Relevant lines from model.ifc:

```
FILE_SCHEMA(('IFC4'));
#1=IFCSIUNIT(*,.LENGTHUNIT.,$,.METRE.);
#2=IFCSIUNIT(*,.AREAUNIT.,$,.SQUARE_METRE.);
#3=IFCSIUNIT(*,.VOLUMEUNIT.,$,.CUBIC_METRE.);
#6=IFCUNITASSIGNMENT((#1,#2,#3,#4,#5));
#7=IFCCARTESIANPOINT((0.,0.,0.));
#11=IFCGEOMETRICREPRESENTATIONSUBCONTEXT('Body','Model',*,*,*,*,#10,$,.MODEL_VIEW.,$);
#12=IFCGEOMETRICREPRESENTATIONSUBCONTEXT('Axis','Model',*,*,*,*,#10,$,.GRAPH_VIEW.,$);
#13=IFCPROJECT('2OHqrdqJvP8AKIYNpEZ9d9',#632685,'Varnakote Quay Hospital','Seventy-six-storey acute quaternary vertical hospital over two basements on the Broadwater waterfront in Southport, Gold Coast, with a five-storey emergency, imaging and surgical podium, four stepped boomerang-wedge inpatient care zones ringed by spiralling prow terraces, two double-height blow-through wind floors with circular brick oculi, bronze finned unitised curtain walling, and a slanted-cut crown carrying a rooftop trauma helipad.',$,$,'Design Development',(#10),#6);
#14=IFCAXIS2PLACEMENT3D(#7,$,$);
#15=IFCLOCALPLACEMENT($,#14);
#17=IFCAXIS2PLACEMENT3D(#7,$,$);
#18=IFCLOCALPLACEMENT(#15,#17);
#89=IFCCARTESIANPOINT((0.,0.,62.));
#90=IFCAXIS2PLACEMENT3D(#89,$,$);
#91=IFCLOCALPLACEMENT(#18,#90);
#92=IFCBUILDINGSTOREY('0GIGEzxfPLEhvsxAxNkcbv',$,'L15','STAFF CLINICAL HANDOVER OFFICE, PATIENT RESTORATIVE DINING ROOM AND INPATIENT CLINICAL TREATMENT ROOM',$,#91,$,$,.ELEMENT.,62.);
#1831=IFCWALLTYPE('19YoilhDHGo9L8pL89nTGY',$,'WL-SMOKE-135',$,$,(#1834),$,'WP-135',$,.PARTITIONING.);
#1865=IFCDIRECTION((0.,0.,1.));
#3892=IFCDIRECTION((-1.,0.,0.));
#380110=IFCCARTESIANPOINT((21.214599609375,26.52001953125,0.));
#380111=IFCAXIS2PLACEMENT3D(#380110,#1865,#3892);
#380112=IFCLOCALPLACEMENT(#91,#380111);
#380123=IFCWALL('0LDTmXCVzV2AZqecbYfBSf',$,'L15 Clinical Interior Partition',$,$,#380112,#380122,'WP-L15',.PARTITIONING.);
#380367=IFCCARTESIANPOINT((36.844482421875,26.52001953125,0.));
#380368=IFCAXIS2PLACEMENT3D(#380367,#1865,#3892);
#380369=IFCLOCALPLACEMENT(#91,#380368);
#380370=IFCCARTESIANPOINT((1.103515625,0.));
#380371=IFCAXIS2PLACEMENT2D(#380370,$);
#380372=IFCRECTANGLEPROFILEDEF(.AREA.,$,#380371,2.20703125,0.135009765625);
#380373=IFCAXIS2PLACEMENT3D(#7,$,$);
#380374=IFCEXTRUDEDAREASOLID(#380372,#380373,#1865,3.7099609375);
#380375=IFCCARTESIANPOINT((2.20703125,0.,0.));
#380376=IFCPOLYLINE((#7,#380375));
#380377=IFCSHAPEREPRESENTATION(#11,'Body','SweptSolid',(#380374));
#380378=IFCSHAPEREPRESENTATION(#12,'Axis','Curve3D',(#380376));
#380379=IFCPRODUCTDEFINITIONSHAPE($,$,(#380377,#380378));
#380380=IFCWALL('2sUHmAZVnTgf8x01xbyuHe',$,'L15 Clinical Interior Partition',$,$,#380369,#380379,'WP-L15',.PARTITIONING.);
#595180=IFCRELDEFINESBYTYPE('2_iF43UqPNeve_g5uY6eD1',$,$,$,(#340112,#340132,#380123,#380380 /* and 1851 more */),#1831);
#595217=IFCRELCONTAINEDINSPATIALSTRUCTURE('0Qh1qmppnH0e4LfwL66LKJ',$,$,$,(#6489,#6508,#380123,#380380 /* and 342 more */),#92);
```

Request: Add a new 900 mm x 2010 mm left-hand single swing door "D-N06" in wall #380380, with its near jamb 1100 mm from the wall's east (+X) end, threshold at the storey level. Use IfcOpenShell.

```python
import numpy as np
import ifcopenshell
import ifcopenshell.api.feature
import ifcopenshell.api.geometry
import ifcopenshell.api.root
import ifcopenshell.api.spatial
import ifcopenshell.geom
import ifcopenshell.util.element
import ifcopenshell.util.placement
import ifcopenshell.util.representation
import ifcopenshell.util.shape
import ifcopenshell.util.unit

model = ifcopenshell.open("model.ifc")
unit_scale = ifcopenshell.util.unit.calculate_unit_scale(model)
settings = ifcopenshell.geom.settings()


def volume(element):
    """Net volume in cubic metres, openings subtracted."""
    shape = ifcopenshell.geom.create_shape(settings, element)
    return ifcopenshell.util.shape.get_volume(shape.geometry)


wall = model.by_id(380380)
storey = ifcopenshell.util.element.get_container(wall, ifc_class="IfcBuildingStorey")
context = ifcopenshell.util.representation.get_context(model, "Model", "Body", "MODEL_VIEW")
before = volume(wall)

width, height, from_end, sill = 0.9, 2.01, 1.1, 0.0  # metres

# The wall runs along its own X axis, and the end named is its -X end.
wall_shape = ifcopenshell.geom.create_shape(settings, wall)
x, y, z = ifcopenshell.util.shape.get_vertices(wall_shape.geometry).T
start = x.min() + from_end
face, thickness = float(y.min()), float(y.max() - y.min())
wall_matrix = ifcopenshell.util.placement.get_local_placement(wall.ObjectPlacement)
level = ifcopenshell.util.placement.get_local_placement(storey.ObjectPlacement)[2, 3]


def in_wall(x, y):
    """Placement at x, y metres in the wall's axes, at sill height."""
    matrix = wall_matrix.copy()
    matrix[:, 3] = wall_matrix @ np.array([x / unit_scale, y / unit_scale, 0.0, 1.0])
    matrix[2, 3] = level + sill / unit_scale
    return matrix


# Opening: a box that overshoots both wall faces by 50 mm.
opening = ifcopenshell.api.root.create_entity(model, ifc_class="IfcOpeningElement", predefined_type="OPENING")
box = ifcopenshell.api.geometry.add_wall_representation(
    model, context=context, length=width, height=height, thickness=thickness + 0.1
)
ifcopenshell.api.geometry.assign_representation(model, product=opening, representation=box)
ifcopenshell.api.geometry.edit_object_placement(model, product=opening, matrix=in_wall(start, face - 0.05), is_si=False)
ifcopenshell.api.feature.add_feature(model, feature=opening, element=wall)

door = ifcopenshell.api.root.create_entity(model, ifc_class="IfcDoor", name="D-N06", predefined_type="DOOR")
door.OverallWidth, door.OverallHeight = width / unit_scale, height / unit_scale
door.OperationType = "SINGLE_SWING_LEFT"
body = ifcopenshell.api.geometry.add_door_representation(
    model,
    context=context,
    overall_width=door.OverallWidth,
    overall_height=door.OverallHeight,
    operation_type="SINGLE_SWING_LEFT",
    lining_properties={"LiningDepth": thickness / unit_scale, "ThresholdDepth": thickness / unit_scale},
)
ifcopenshell.api.geometry.assign_representation(model, product=door, representation=body)
ifcopenshell.api.spatial.assign_container(model, products=[door], relating_structure=storey)
ifcopenshell.api.feature.add_filling(model, opening=opening, element=door)

# The lining spans the wall, so the door starts at the wall face.
ifcopenshell.api.geometry.edit_object_placement(model, product=door, matrix=in_wall(start, face), is_si=False)

after = volume(wall)

print(f"wall volume {before:.3f} -> {after:.3f} m3")

model.write("model_updated.ifc")
```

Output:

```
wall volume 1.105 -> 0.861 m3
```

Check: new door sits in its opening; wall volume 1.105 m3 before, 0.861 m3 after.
